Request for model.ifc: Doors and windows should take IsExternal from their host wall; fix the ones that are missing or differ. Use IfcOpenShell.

First a look at what the model holds.

```python
import ifcopenshell
import ifcopenshell.util.element

model = ifcopenshell.open("model.ifc")
print(model.schema)
seen = {}
for e in model.by_type("IfcDoor") + model.by_type("IfcWindow"):
    if not e.FillsVoids:
        continue
    host = e.FillsVoids[0].RelatingOpeningElement.VoidsElements[0].RelatingBuildingElement
    own = ifcopenshell.util.element.get_pset(e, f"Pset_{e.is_a()[3:].removesuffix('StandardCase')}Common", "IsExternal")
    wall = ifcopenshell.util.element.get_pset(host, "Pset_WallCommon", "IsExternal")
    seen[e.is_a(), own, wall] = seen.get((e.is_a(), own, wall), 0) + 1
for (cls, own, wall), count in sorted(seen.items(), key=str):
    print(count, cls, "IsExternal:", own, "| host wall:", wall)
```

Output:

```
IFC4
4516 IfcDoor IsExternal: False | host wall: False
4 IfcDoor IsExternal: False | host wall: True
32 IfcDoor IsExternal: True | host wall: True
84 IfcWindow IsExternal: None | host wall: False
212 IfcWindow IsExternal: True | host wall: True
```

```python
import ifcopenshell
import ifcopenshell.api.pset
import ifcopenshell.util.element

model = ifcopenshell.open("model.ifc")

count = 0
for ifc_class, pset_name in (("IfcDoor", "Pset_DoorCommon"), ("IfcWindow", "Pset_WindowCommon")):
    for e in model.by_type(ifc_class):
        if not e.FillsVoids:
            continue
        host = e.FillsVoids[0].RelatingOpeningElement.VoidsElements[0].RelatingBuildingElement
        external = ifcopenshell.util.element.get_pset(host, "Pset_WallCommon", "IsExternal")
        if external is None or ifcopenshell.util.element.get_pset(e, pset_name, "IsExternal") == external:
            continue
        found = ifcopenshell.util.element.get_pset(e, pset_name, should_inherit=False)
        if found:
            pset = model.by_id(found["id"])
            if len(ifcopenshell.util.element.get_elements_by_pset(pset)) > 1:
                pset = ifcopenshell.api.pset.unshare_pset(model, products=[e], pset=pset)[0]
        else:
            pset = ifcopenshell.api.pset.add_pset(model, product=e, name=pset_name)
        ifcopenshell.api.pset.edit_pset(model, pset=pset, properties={"IsExternal": external})
        count += 1

print(count, "updated")

model.write("model_updated.ifc")
```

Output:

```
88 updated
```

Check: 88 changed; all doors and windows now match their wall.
